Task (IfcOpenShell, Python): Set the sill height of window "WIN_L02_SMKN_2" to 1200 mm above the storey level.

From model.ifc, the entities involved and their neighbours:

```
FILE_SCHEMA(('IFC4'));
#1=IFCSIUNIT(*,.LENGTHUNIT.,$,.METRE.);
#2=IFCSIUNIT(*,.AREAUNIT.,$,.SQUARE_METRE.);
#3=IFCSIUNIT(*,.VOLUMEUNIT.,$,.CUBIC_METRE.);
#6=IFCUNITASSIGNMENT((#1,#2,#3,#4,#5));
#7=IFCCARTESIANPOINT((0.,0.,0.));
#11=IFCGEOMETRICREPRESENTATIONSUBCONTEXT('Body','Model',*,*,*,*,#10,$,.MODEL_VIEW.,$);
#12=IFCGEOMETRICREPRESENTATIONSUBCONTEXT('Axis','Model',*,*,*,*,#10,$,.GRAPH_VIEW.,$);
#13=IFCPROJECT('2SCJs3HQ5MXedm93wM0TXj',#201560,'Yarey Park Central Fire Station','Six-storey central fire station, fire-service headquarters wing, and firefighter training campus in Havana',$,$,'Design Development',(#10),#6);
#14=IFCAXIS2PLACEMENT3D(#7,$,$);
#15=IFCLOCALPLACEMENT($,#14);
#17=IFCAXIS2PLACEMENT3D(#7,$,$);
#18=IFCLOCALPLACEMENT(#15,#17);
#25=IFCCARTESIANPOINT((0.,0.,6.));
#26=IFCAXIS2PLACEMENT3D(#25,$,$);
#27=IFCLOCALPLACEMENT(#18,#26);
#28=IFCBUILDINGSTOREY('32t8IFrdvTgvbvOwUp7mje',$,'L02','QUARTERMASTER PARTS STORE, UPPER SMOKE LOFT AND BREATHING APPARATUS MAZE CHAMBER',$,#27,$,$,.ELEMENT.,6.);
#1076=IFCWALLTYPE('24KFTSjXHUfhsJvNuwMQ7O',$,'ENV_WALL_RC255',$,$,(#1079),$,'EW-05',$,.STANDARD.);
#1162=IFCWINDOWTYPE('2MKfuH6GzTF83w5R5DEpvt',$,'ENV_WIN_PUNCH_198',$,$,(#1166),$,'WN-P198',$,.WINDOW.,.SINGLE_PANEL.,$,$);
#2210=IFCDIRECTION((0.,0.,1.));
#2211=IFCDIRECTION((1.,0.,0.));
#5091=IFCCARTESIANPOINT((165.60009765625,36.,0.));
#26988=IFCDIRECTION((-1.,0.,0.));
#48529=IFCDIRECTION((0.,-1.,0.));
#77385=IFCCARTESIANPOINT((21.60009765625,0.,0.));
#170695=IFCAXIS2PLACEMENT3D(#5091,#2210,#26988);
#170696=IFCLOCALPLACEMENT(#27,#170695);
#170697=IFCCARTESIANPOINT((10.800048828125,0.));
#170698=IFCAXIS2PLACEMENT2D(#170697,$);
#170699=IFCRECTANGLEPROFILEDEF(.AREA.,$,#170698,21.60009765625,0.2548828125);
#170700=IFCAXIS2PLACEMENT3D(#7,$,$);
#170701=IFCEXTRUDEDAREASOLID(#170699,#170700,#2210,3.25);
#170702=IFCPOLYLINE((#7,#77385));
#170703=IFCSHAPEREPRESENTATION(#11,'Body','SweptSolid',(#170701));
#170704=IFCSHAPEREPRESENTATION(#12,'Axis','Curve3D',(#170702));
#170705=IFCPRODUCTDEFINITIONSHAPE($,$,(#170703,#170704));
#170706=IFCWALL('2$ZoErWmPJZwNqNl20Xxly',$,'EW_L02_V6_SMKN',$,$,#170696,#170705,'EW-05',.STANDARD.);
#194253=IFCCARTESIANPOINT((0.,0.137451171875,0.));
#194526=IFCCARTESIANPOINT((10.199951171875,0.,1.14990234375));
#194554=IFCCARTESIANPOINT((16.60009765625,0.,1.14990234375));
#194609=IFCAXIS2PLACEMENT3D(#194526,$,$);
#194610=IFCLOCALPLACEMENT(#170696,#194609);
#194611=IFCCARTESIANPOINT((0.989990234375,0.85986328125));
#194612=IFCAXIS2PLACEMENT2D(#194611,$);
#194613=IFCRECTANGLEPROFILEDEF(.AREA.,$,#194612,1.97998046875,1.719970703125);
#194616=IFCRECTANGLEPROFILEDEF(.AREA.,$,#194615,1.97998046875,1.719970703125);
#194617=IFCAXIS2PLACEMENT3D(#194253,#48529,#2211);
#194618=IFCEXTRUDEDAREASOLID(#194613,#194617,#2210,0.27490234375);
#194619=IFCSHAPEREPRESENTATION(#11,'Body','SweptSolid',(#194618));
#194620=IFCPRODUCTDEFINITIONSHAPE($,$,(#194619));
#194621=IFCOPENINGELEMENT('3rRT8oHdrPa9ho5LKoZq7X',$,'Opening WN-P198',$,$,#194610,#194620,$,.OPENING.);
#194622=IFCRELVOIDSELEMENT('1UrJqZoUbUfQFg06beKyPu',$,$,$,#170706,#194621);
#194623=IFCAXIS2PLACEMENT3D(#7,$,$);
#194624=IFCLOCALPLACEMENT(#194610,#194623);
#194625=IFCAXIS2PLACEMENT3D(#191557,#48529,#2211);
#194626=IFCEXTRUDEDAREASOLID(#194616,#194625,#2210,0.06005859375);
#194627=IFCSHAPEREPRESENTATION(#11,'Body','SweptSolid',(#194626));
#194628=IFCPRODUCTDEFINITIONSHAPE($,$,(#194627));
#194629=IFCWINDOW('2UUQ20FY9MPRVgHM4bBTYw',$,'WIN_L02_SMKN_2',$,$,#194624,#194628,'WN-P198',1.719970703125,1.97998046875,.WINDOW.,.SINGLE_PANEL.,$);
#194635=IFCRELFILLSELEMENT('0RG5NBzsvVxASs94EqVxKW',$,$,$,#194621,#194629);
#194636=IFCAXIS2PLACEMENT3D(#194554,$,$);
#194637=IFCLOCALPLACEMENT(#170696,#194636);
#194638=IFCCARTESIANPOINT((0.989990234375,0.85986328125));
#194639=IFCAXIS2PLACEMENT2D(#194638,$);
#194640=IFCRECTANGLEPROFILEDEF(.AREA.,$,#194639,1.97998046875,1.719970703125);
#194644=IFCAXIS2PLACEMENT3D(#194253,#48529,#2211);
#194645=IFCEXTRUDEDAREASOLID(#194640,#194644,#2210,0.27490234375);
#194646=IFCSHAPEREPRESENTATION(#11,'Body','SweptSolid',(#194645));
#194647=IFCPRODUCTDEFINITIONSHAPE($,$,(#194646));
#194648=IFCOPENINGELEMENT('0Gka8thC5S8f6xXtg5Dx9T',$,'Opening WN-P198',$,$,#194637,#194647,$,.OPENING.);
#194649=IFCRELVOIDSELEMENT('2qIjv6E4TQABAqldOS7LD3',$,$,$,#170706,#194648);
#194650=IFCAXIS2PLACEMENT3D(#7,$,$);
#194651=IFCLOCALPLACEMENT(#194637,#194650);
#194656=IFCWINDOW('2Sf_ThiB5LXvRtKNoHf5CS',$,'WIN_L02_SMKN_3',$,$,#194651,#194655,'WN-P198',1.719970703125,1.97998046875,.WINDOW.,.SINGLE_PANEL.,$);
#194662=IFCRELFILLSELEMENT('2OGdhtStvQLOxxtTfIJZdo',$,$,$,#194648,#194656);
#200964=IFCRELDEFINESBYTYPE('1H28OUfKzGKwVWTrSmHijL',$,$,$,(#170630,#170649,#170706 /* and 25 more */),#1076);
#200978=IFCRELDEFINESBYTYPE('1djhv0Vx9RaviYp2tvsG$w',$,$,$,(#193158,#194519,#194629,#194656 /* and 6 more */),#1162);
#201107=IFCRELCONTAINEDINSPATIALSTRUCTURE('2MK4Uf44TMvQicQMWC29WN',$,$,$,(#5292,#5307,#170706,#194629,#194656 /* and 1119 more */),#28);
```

```python
import numpy as np
import ifcopenshell
import ifcopenshell.api.geometry
import ifcopenshell.geom
import ifcopenshell.util.element
import ifcopenshell.util.placement
import ifcopenshell.util.shape
import ifcopenshell.util.unit

model = ifcopenshell.open("model.ifc")
unit_scale = ifcopenshell.util.unit.calculate_unit_scale(model)

window = model.by_guid("2UUQ20FY9MPRVgHM4bBTYw")
opening = window.FillsVoids[0].RelatingOpeningElement
storey = ifcopenshell.util.element.get_container(window, ifc_class="IfcBuildingStorey")
level = ifcopenshell.util.placement.get_local_placement(storey.ObjectPlacement)[2, 3]

# The opening's origin need not be at the sill, so measure its lowest point.
shape = ifcopenshell.geom.create_shape(ifcopenshell.geom.settings(), opening)
bottom = ifcopenshell.util.shape.get_shape_bottom_elevation(shape, shape.geometry) / unit_scale
dz = level + 1.2 / unit_scale - bottom

shift = np.array([0.0, 0.0, dz])
# The window is placed relative to its opening, so it follows when the opening moves.
matrix = ifcopenshell.util.placement.get_local_placement(opening.ObjectPlacement)
matrix[:3, 3] += shift
ifcopenshell.api.geometry.edit_object_placement(
    model, product=opening, matrix=matrix, is_si=False, should_transform_children=True
)

print(f"moved by {dz * unit_scale:+.3f} m")

model.write("model_rev.ifc")
```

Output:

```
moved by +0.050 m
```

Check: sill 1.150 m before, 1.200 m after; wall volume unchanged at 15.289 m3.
